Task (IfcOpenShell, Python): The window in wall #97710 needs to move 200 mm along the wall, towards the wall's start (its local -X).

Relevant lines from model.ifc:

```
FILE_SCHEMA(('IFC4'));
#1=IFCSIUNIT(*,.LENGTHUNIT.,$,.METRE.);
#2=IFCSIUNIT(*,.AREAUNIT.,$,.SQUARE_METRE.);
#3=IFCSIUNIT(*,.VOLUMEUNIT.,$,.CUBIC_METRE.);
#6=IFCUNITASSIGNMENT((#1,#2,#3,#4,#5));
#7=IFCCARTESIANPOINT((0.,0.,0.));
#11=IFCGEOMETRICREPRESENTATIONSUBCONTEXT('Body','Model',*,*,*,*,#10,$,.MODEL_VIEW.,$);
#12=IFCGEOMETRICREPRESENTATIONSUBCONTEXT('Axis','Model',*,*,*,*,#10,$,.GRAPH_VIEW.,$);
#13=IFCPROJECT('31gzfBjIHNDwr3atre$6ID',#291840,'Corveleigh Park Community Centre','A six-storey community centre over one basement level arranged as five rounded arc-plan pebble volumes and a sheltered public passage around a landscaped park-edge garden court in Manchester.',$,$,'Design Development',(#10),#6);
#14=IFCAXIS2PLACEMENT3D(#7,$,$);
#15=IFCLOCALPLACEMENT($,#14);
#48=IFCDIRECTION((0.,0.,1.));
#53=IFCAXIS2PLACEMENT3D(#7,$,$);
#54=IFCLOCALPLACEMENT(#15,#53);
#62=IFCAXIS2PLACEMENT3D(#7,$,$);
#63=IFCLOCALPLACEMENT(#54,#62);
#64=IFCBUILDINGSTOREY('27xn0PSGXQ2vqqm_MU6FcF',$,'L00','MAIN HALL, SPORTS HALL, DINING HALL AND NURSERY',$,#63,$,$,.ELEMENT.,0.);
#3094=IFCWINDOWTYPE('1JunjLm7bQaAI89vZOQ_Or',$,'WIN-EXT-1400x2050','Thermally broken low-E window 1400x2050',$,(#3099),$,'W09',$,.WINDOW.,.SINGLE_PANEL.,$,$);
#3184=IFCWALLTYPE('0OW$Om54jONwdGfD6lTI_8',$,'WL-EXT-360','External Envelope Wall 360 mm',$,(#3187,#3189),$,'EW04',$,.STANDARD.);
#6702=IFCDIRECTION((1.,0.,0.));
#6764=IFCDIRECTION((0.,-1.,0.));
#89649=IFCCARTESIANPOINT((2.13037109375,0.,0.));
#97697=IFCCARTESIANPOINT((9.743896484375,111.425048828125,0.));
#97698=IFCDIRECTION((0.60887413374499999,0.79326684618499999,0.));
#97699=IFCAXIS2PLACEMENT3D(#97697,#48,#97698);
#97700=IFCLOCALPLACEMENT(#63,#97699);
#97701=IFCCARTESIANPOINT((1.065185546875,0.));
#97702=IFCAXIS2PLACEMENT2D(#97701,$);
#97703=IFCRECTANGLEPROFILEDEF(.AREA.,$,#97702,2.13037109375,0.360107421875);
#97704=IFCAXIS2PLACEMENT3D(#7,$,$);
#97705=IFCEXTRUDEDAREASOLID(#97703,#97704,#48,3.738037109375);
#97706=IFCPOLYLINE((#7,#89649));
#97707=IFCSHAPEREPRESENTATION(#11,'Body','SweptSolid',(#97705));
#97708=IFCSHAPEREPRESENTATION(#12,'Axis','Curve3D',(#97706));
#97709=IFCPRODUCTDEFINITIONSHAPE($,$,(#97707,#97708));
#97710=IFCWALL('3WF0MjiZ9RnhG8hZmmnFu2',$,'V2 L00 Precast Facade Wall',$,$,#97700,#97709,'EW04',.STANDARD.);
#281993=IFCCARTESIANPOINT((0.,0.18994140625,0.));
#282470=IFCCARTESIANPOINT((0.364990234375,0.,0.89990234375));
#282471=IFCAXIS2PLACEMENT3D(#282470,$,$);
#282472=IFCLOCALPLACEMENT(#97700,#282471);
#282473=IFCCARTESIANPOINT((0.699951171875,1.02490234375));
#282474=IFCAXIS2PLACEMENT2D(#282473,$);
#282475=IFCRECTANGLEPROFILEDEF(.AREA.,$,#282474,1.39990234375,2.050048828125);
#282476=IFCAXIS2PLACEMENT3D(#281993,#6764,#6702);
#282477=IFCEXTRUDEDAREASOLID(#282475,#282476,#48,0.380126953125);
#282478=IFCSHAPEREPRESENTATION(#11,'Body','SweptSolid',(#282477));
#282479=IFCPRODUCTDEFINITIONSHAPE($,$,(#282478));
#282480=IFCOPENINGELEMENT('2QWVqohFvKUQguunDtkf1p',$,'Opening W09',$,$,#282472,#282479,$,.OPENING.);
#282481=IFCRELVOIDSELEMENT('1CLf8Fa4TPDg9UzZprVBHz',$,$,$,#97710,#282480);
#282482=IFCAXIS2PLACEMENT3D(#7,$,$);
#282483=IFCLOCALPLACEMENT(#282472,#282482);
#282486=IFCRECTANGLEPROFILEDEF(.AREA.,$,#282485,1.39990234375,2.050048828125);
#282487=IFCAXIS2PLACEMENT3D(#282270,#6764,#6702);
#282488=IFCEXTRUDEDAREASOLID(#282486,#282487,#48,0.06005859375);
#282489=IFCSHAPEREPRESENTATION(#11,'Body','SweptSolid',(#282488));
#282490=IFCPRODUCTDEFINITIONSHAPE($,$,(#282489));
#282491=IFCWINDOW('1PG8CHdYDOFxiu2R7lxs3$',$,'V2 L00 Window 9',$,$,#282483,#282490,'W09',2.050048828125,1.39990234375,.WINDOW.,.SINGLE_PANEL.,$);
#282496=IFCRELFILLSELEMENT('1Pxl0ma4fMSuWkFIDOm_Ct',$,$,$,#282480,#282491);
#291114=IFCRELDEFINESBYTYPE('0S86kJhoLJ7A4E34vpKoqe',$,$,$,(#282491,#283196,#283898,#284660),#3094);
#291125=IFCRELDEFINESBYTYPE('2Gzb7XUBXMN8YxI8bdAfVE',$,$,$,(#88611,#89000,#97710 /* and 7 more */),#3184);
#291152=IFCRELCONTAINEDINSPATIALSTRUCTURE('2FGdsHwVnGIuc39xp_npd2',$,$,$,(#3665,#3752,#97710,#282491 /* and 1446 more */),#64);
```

```python
import ifcopenshell
import ifcopenshell.api.geometry
import ifcopenshell.util.placement

model = ifcopenshell.open("model.ifc")

window = model.by_guid("1PG8CHdYDOFxiu2R7lxs3$")
opening = window.FillsVoids[0].RelatingOpeningElement
wall = opening.VoidsElements[0].RelatingBuildingElement

wall_matrix = ifcopenshell.util.placement.get_local_placement(wall.ObjectPlacement)
shift = wall_matrix[:3, 0] * -0.2
before = ifcopenshell.util.placement.get_local_placement(window.ObjectPlacement)[:3, 3].copy()

# The window is placed relative to its opening, so it follows when the opening moves.
matrix = ifcopenshell.util.placement.get_local_placement(opening.ObjectPlacement)
matrix[:3, 3] += shift
ifcopenshell.api.geometry.edit_object_placement(
    model, product=opening, matrix=matrix, is_si=False, should_transform_children=True
)

after = ifcopenshell.util.placement.get_local_placement(window.ObjectPlacement)[:3, 3]
print("window moved by", (after - before).round(3) + 0.0)

model.write("model_rev.ifc")
```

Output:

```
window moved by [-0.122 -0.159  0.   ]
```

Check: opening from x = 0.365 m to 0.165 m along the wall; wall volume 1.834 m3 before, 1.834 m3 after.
